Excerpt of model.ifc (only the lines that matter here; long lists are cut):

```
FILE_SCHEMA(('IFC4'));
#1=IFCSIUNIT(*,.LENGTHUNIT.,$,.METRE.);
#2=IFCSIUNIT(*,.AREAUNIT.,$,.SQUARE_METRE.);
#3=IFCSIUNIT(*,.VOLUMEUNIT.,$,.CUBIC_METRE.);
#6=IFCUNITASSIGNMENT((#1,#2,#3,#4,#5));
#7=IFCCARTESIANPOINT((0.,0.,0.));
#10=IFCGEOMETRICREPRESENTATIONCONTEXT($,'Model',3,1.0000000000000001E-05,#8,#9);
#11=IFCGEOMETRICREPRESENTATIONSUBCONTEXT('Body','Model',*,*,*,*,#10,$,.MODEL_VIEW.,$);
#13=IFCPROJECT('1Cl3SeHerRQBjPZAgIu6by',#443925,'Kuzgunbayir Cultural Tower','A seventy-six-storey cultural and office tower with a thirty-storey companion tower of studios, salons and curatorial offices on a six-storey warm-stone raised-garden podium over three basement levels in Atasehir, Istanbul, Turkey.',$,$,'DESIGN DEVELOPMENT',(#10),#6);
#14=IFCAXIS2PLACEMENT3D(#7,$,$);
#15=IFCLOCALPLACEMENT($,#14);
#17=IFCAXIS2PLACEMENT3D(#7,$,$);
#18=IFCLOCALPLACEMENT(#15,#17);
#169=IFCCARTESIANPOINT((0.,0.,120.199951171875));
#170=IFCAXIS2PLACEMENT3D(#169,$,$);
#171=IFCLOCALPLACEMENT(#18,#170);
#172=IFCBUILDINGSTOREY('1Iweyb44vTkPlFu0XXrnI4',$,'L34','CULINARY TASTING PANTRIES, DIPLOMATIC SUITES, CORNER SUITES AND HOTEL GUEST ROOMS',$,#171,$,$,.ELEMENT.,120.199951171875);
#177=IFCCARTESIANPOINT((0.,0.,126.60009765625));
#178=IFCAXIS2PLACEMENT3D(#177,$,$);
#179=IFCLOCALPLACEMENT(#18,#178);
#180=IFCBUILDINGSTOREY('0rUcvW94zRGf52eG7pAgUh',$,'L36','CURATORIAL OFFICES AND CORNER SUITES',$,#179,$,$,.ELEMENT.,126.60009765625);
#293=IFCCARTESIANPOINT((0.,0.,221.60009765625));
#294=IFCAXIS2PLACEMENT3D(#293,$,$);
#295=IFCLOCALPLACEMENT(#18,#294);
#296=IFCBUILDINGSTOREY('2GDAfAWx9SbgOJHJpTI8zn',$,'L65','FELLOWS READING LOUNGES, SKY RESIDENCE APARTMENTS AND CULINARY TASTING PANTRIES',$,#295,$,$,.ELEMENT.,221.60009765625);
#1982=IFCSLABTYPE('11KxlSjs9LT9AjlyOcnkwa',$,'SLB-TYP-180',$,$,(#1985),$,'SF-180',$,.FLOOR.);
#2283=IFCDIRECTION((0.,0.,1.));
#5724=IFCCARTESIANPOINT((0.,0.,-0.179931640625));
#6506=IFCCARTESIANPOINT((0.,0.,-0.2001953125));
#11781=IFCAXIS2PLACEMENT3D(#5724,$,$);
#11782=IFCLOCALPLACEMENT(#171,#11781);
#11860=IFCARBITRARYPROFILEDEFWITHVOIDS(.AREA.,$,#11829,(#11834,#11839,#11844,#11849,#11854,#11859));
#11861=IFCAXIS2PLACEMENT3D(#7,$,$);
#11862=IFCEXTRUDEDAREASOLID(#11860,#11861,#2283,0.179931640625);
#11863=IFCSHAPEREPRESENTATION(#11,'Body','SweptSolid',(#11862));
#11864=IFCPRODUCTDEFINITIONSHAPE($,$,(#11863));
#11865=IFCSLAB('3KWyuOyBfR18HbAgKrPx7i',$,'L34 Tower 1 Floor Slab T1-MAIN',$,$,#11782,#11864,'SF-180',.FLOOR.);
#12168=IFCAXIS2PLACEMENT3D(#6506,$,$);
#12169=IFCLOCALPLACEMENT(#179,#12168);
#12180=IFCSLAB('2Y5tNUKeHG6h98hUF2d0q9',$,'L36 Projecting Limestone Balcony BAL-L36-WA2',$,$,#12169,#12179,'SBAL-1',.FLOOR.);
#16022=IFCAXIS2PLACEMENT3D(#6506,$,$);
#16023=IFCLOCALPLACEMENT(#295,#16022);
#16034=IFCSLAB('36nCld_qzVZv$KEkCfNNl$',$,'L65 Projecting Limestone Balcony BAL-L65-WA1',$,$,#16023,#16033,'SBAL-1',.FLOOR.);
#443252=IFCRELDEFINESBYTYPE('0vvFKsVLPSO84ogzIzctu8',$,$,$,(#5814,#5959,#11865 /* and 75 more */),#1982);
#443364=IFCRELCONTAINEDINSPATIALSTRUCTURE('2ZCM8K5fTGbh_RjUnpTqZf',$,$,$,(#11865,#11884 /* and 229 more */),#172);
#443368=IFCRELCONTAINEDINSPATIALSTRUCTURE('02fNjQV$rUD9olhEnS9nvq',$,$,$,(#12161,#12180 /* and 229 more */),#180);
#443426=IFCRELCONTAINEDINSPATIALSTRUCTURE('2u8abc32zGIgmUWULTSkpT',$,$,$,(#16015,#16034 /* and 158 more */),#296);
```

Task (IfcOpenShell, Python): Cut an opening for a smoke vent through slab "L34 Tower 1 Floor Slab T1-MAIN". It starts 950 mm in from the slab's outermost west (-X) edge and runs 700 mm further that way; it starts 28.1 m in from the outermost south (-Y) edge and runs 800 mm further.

```python
import numpy as np
import ifcopenshell
import ifcopenshell.api.feature
import ifcopenshell.api.geometry
import ifcopenshell.api.root
import ifcopenshell.geom
import ifcopenshell.util.placement
import ifcopenshell.util.representation
import ifcopenshell.util.shape
import ifcopenshell.util.unit

model = ifcopenshell.open("model.ifc")
unit_scale = ifcopenshell.util.unit.calculate_unit_scale(model)
settings = ifcopenshell.geom.settings()


def volume(element):
    """Net volume in cubic metres, openings subtracted."""
    shape = ifcopenshell.geom.create_shape(settings, element)
    return ifcopenshell.util.shape.get_volume(shape.geometry)


slab = model.by_id(11865)
before = volume(slab)

# Extent in the slab's own axes, in metres. The edges named are its -X and -Y sides.
slab_shape = ifcopenshell.geom.create_shape(settings, slab)
vertices = ifcopenshell.util.shape.get_vertices(slab_shape.geometry)
x_min, y_min, bottom = vertices.min(axis=0)
top = vertices[:, 2].max()

opening = ifcopenshell.api.root.create_entity(model, ifc_class="IfcOpeningElement", name="Smoke vent opening", predefined_type="OPENING")
context = ifcopenshell.util.representation.get_context(model, "Model", "Body", "MODEL_VIEW")
width, depth = 0.7, 0.8
outline = [(0.0, 0.0), (width, 0.0), (width, depth), (0.0, depth), (0.0, 0.0)]
# Overshoot both faces by 50 mm so the cut is clean.
shape = ifcopenshell.api.geometry.add_slab_representation(
    model, context=context, depth=top - bottom + 0.1, polyline=outline
)
ifcopenshell.api.geometry.assign_representation(model, product=opening, representation=shape)

matrix = ifcopenshell.util.placement.get_local_placement(slab.ObjectPlacement)
matrix[:, 3] = matrix @ np.append(np.array([x_min + 0.95, y_min + 28.1, bottom - 0.05]) / unit_scale, 1.0)
ifcopenshell.api.geometry.edit_object_placement(model, product=opening, matrix=matrix, is_si=False)
ifcopenshell.api.feature.add_feature(model, feature=opening, element=slab)

after = volume(slab)

print(f"slab volume {before:.3f} -> {after:.3f} m3")

model.write("model-out.ifc")
```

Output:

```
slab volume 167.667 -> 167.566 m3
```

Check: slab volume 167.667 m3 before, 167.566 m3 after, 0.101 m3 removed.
